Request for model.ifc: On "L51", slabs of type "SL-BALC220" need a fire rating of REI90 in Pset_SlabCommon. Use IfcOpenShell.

First a look at what the model holds.

```python
import ifcopenshell
import ifcopenshell.util.element

model = ifcopenshell.open("model.ifc")
print(model.schema)
storey = next(s for s in model.by_type("IfcBuildingStorey") if s.Name == "L51")
slabs = [e for e in ifcopenshell.util.element.get_decomposition(storey) if e.is_a("IfcSlab")]
seen = {}
for e in slabs:
    element_type = ifcopenshell.util.element.get_type(e)
    key = (element_type.Name if element_type != e and element_type else None, ifcopenshell.util.element.get_pset(e, "Pset_SlabCommon", "FireRating"))
    seen[key] = seen.get(key, 0) + 1
for (name, value), count in sorted(seen.items(), key=str):
    print(count, "x", name, "|", value)
```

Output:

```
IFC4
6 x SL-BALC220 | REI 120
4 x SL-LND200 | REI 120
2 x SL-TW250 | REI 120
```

```python
import ifcopenshell
import ifcopenshell.api.pset
import ifcopenshell.util.element

model = ifcopenshell.open("model.ifc")

storey = next(s for s in model.by_type("IfcBuildingStorey") if s.Name == "L51")
slabs = [e for e in ifcopenshell.util.element.get_decomposition(storey) if e.is_a("IfcSlab")]

count = 0
for e in slabs:
    element_type = ifcopenshell.util.element.get_type(e)
    if element_type in (None, e) or element_type.Name != "SL-BALC220":
        continue
    found = ifcopenshell.util.element.get_pset(e, "Pset_SlabCommon", should_inherit=False)
    if found:
        pset = model.by_id(found["id"])
        if len(ifcopenshell.util.element.get_elements_by_pset(pset)) > 1:
            pset = ifcopenshell.api.pset.unshare_pset(model, products=[e], pset=pset)[0]
    else:
        pset = ifcopenshell.api.pset.add_pset(model, product=e, name="Pset_SlabCommon")
    ifcopenshell.api.pset.edit_pset(model, pset=pset, properties={"FireRating": "REI90"})
    count += 1

print(count, "slabs updated")

model.write("model_v2.ifc")
```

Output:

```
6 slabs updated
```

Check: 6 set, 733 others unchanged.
